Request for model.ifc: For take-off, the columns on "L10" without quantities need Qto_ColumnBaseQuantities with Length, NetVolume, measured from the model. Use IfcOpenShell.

First a look at what the model holds.

```python
import ifcopenshell
import ifcopenshell.util.element
import ifcopenshell.util.unit

model = ifcopenshell.open("model.ifc")
print(model.schema)
for unit_type in ("LENGTHUNIT", "AREAUNIT", "VOLUMEUNIT"):
    print(unit_type, ifcopenshell.util.unit.calculate_unit_scale(model, unit_type))
storey = next(s for s in model.by_type("IfcBuildingStorey") if s.Name == "L10")
columns = [e for e in ifcopenshell.util.element.get_decomposition(storey) if e.is_a("IfcColumn")]
for e in sorted(columns, key=lambda e: e.id()):
    print(e.id(), e.is_a(), e.Name, list(ifcopenshell.util.element.get_psets(e, qtos_only=True)), sep=" | ")
```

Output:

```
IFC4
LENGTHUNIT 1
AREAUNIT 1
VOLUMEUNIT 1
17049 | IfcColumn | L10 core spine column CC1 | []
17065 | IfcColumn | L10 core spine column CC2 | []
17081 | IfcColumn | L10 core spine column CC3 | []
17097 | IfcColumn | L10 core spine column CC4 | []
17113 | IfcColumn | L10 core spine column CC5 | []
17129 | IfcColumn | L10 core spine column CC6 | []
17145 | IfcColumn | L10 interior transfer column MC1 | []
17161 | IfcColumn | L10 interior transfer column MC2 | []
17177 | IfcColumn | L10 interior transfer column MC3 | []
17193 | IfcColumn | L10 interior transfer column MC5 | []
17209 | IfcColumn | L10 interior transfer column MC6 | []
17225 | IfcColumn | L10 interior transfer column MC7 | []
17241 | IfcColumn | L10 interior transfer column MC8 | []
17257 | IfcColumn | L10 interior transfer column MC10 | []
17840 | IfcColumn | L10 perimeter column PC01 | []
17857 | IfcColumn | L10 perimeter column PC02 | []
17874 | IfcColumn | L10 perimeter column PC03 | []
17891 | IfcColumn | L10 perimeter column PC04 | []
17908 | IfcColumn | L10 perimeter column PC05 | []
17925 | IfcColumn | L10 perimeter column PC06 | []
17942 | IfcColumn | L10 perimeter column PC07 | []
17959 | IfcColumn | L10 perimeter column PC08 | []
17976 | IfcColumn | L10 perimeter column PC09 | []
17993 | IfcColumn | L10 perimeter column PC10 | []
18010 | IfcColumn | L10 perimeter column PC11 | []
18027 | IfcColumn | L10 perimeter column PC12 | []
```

```python
import ifcopenshell
import ifcopenshell.api.pset
import ifcopenshell.geom
import ifcopenshell.util.element
import ifcopenshell.util.shape
import ifcopenshell.util.unit

model = ifcopenshell.open("model.ifc")
unit_scale = ifcopenshell.util.unit.calculate_unit_scale(model)
volume_scale = ifcopenshell.util.unit.calculate_unit_scale(model, "VOLUMEUNIT")
settings = ifcopenshell.geom.settings()

storey = next(s for s in model.by_type("IfcBuildingStorey") if s.Name == "L10")
columns = [e for e in ifcopenshell.util.element.get_decomposition(storey) if e.is_a("IfcColumn")]

for e in sorted(columns, key=lambda e: e.id()):
    if ifcopenshell.util.element.get_psets(e, qtos_only=True, should_inherit=False):
        continue
    # Geometry comes back in metres, in the element's own axes.
    shape = ifcopenshell.geom.create_shape(settings, e)
    values = {
        "Length": ifcopenshell.util.shape.get_z(shape.geometry) / unit_scale,
        "NetVolume": ifcopenshell.util.shape.get_volume(shape.geometry) / volume_scale,
    }
    qto = ifcopenshell.api.pset.add_qto(model, product=e, name="Qto_ColumnBaseQuantities")
    ifcopenshell.api.pset.edit_qto(model, qto=qto, properties=values)
    print(e.id(), {k: round(v, 3) for k, v in values.items()})

model.write("model_updated.ifc")
```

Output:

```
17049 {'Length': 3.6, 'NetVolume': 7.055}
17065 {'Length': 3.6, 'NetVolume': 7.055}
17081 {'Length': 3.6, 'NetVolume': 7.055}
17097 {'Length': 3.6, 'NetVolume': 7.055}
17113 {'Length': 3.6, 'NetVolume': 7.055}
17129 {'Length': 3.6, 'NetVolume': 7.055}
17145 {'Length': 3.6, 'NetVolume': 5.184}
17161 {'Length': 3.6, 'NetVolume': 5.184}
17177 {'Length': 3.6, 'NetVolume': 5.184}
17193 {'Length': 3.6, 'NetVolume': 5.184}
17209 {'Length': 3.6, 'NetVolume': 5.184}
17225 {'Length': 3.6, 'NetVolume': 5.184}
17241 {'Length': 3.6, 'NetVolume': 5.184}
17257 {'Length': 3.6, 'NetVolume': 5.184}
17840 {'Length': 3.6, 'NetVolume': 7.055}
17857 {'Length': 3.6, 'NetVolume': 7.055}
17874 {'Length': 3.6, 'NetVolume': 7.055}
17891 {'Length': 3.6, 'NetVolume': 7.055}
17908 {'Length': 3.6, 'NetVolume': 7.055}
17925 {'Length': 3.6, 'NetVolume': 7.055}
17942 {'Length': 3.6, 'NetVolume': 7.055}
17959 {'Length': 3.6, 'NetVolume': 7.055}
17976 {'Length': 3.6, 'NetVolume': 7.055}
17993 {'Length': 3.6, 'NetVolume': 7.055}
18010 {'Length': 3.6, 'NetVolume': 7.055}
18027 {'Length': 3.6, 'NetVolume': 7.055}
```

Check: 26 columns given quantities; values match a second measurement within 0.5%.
